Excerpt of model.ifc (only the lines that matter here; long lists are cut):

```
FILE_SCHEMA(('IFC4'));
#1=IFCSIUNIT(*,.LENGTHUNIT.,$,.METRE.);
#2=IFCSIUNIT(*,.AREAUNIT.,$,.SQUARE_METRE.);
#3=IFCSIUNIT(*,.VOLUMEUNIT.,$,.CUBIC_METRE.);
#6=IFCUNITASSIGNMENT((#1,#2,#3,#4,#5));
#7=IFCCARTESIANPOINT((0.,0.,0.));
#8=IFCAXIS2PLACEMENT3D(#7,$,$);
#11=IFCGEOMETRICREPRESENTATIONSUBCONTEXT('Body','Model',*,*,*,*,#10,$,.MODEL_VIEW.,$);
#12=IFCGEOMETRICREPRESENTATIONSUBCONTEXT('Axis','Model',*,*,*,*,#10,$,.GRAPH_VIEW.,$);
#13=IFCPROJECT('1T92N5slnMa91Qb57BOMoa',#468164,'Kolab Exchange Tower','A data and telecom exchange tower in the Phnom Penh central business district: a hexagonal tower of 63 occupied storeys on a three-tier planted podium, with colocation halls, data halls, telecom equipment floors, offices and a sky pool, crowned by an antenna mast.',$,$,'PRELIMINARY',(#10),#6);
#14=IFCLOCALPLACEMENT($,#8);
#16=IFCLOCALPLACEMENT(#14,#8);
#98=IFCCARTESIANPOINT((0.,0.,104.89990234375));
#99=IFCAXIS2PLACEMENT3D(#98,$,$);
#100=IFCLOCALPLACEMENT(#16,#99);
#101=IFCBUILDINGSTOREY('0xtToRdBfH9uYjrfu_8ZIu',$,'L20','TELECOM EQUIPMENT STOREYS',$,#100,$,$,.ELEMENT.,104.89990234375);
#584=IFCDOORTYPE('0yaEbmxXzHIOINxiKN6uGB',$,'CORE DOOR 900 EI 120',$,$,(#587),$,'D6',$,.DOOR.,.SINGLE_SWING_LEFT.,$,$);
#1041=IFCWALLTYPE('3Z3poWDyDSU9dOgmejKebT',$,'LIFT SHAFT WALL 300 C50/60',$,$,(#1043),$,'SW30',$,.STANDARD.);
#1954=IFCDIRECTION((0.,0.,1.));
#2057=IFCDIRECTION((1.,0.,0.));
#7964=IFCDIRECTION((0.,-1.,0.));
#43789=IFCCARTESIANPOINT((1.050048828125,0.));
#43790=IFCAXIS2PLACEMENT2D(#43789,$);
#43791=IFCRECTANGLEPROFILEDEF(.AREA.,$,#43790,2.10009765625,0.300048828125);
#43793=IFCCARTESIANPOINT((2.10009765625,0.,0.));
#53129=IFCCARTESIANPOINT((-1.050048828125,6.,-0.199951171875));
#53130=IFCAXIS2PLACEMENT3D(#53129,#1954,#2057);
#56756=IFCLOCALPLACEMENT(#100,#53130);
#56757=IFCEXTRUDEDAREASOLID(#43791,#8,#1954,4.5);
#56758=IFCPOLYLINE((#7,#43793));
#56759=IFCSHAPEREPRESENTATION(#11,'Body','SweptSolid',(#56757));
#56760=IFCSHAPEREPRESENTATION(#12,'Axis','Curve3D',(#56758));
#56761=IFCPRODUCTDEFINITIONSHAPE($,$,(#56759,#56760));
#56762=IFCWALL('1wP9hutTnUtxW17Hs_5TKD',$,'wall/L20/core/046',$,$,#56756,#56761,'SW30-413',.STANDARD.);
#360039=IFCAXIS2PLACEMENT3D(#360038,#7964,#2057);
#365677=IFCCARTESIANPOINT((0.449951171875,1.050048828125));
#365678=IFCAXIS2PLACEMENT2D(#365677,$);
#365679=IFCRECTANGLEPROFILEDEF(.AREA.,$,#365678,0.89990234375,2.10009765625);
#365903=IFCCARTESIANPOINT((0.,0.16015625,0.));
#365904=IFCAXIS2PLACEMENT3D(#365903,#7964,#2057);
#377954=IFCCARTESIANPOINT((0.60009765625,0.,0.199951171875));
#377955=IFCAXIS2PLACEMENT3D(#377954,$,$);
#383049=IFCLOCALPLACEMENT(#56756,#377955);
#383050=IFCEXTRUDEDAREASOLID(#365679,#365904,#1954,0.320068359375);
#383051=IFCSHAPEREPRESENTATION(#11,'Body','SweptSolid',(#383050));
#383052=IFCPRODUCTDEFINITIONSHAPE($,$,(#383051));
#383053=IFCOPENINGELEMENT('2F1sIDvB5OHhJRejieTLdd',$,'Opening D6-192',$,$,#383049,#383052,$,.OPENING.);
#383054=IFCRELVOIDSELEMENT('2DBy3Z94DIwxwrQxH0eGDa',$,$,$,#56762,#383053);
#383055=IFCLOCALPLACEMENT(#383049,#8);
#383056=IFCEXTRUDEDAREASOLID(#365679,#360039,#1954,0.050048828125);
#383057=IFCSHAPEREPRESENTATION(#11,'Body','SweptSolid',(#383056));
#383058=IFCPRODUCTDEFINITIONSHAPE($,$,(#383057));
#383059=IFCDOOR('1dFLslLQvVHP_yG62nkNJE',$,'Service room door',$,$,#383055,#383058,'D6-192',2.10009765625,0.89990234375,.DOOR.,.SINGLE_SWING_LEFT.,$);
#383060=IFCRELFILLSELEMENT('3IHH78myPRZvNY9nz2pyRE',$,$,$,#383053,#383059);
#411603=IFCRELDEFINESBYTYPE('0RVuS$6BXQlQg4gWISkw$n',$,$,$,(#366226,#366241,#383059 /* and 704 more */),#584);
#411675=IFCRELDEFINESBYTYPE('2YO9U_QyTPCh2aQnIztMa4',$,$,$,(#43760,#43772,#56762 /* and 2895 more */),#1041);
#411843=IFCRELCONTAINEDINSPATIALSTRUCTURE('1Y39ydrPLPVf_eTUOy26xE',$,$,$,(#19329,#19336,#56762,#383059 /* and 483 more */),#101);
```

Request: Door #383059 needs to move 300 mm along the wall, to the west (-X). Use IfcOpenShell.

```python
import ifcopenshell
import ifcopenshell.api.geometry
import ifcopenshell.util.placement
import ifcopenshell.util.unit

model = ifcopenshell.open("model.ifc")
unit_scale = ifcopenshell.util.unit.calculate_unit_scale(model)

door = model.by_guid("1dFLslLQvVHP_yG62nkNJE")
opening = door.FillsVoids[0].RelatingOpeningElement
wall = opening.VoidsElements[0].RelatingBuildingElement

wall_matrix = ifcopenshell.util.placement.get_local_placement(wall.ObjectPlacement)
shift = wall_matrix[:3, 0] * -0.3 / unit_scale
before = ifcopenshell.util.placement.get_local_placement(door.ObjectPlacement)[:3, 3].copy()

# The door is placed relative to its opening, so it follows when the opening moves.
matrix = ifcopenshell.util.placement.get_local_placement(opening.ObjectPlacement)
matrix[:3, 3] += shift
ifcopenshell.api.geometry.edit_object_placement(
    model, product=opening, matrix=matrix, is_si=False, should_transform_children=True
)

after = ifcopenshell.util.placement.get_local_placement(door.ObjectPlacement)[:3, 3]
print("door moved by", (after - before).round(3) + 0.0)

model.write("model_edited.ifc")
```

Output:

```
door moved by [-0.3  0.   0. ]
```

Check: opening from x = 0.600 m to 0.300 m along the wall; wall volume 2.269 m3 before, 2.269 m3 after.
